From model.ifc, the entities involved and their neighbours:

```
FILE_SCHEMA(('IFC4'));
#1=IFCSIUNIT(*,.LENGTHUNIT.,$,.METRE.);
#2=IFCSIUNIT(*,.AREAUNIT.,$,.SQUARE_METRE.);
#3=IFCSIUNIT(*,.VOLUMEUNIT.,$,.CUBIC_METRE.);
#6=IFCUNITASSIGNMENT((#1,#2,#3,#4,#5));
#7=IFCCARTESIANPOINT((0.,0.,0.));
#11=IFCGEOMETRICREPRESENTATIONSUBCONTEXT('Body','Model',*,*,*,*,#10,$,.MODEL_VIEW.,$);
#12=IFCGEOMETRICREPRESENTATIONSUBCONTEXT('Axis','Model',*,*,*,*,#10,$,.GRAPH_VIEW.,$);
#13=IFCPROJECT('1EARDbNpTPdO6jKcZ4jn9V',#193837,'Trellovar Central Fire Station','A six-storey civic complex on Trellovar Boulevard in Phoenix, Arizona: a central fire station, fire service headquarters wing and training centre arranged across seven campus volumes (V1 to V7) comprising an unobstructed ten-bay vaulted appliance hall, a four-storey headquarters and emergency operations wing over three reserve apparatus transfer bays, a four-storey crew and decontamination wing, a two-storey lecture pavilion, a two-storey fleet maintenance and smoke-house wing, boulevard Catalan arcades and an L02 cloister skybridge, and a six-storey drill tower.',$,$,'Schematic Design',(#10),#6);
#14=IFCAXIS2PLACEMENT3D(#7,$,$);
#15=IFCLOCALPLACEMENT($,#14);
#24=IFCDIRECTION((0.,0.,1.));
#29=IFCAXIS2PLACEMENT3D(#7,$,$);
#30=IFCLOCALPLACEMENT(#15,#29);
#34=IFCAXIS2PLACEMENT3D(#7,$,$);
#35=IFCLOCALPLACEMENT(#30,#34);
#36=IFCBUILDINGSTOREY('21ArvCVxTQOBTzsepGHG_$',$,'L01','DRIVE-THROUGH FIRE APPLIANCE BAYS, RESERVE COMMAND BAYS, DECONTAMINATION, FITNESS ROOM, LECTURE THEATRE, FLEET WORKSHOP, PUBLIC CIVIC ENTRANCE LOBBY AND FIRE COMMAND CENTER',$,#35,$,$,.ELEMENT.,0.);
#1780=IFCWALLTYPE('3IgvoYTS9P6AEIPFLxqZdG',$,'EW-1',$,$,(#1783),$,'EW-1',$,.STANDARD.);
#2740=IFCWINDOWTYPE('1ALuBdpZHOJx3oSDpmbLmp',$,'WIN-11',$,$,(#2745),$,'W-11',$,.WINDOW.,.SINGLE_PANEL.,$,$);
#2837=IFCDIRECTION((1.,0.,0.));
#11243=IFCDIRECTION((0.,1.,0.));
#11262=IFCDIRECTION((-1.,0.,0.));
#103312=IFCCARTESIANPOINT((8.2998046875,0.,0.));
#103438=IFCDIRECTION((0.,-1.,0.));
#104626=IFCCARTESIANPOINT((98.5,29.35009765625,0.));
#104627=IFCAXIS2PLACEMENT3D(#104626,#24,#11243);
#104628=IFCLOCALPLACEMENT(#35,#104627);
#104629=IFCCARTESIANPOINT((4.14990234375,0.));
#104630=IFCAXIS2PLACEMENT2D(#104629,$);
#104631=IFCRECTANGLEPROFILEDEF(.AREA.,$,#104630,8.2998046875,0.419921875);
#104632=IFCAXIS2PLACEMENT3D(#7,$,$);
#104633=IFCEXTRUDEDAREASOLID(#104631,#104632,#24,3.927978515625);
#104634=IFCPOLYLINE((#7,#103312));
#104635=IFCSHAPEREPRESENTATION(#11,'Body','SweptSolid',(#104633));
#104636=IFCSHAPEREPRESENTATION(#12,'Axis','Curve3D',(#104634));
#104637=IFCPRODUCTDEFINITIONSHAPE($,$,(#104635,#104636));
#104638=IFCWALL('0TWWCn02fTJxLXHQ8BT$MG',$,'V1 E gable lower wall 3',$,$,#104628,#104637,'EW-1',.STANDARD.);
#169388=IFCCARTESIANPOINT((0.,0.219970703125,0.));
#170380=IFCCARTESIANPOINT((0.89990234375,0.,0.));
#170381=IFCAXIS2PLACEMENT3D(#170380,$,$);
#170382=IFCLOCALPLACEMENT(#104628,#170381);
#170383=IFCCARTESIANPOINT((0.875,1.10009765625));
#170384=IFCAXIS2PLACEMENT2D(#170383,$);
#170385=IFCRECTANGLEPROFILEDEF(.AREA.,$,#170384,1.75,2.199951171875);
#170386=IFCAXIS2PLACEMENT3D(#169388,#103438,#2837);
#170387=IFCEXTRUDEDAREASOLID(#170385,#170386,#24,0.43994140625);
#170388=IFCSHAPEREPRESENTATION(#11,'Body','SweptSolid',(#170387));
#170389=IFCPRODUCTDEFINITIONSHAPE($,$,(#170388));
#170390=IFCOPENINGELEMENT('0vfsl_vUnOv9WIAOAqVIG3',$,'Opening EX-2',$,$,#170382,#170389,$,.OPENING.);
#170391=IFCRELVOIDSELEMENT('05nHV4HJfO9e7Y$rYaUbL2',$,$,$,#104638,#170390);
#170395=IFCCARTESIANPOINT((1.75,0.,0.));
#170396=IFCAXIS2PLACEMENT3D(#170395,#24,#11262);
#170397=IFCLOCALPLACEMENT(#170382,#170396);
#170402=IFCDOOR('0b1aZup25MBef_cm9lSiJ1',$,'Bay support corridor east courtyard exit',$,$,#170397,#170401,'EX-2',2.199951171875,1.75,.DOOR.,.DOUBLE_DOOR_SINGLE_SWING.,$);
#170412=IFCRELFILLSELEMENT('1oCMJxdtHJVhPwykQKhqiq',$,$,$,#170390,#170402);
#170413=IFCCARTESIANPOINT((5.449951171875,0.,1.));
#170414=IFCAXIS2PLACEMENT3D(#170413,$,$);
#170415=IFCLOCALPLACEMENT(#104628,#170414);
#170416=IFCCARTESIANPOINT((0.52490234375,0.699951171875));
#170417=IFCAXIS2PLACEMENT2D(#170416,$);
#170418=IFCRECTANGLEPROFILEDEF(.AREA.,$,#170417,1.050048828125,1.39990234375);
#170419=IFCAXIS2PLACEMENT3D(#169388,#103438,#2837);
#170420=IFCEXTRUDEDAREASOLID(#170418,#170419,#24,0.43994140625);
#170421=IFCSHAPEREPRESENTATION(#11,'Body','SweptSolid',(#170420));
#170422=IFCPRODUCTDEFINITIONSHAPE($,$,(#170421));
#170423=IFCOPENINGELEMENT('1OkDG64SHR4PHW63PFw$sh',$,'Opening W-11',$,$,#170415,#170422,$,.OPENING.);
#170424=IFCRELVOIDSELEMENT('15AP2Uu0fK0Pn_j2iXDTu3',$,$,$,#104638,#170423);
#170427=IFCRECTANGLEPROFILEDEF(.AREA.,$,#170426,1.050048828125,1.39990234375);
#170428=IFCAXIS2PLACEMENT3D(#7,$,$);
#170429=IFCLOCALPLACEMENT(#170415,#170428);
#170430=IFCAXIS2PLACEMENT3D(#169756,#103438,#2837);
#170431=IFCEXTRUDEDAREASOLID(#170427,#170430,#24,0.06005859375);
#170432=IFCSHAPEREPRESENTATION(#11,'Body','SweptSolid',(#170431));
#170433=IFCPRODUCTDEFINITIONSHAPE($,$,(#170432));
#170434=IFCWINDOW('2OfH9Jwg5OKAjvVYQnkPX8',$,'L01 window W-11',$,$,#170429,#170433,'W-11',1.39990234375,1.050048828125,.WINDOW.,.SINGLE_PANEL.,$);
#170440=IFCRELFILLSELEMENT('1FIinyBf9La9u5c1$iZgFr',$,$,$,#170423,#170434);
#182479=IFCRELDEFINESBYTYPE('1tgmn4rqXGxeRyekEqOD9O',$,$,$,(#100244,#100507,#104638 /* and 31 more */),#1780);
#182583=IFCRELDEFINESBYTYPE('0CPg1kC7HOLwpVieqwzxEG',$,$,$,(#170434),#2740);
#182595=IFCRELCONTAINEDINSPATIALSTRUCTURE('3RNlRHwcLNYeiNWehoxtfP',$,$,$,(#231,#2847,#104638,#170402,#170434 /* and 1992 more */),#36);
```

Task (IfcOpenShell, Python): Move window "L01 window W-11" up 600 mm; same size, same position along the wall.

```python
import numpy as np
import ifcopenshell
import ifcopenshell.api.geometry
import ifcopenshell.util.placement
import ifcopenshell.util.unit

model = ifcopenshell.open("model.ifc")
unit_scale = ifcopenshell.util.unit.calculate_unit_scale(model)

window = model.by_guid("2OfH9Jwg5OKAjvVYQnkPX8")
opening = window.FillsVoids[0].RelatingOpeningElement
dz = 0.6

shift = np.array([0.0, 0.0, dz])
# The window is placed relative to its opening, so it follows when the opening moves.
matrix = ifcopenshell.util.placement.get_local_placement(opening.ObjectPlacement)
matrix[:3, 3] += shift
ifcopenshell.api.geometry.edit_object_placement(
    model, product=opening, matrix=matrix, is_si=False, should_transform_children=True
)

print(f"moved by {dz * unit_scale:+.3f} m")

model.write("model_v2.ifc")
```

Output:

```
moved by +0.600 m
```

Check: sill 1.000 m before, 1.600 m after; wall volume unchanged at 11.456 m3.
